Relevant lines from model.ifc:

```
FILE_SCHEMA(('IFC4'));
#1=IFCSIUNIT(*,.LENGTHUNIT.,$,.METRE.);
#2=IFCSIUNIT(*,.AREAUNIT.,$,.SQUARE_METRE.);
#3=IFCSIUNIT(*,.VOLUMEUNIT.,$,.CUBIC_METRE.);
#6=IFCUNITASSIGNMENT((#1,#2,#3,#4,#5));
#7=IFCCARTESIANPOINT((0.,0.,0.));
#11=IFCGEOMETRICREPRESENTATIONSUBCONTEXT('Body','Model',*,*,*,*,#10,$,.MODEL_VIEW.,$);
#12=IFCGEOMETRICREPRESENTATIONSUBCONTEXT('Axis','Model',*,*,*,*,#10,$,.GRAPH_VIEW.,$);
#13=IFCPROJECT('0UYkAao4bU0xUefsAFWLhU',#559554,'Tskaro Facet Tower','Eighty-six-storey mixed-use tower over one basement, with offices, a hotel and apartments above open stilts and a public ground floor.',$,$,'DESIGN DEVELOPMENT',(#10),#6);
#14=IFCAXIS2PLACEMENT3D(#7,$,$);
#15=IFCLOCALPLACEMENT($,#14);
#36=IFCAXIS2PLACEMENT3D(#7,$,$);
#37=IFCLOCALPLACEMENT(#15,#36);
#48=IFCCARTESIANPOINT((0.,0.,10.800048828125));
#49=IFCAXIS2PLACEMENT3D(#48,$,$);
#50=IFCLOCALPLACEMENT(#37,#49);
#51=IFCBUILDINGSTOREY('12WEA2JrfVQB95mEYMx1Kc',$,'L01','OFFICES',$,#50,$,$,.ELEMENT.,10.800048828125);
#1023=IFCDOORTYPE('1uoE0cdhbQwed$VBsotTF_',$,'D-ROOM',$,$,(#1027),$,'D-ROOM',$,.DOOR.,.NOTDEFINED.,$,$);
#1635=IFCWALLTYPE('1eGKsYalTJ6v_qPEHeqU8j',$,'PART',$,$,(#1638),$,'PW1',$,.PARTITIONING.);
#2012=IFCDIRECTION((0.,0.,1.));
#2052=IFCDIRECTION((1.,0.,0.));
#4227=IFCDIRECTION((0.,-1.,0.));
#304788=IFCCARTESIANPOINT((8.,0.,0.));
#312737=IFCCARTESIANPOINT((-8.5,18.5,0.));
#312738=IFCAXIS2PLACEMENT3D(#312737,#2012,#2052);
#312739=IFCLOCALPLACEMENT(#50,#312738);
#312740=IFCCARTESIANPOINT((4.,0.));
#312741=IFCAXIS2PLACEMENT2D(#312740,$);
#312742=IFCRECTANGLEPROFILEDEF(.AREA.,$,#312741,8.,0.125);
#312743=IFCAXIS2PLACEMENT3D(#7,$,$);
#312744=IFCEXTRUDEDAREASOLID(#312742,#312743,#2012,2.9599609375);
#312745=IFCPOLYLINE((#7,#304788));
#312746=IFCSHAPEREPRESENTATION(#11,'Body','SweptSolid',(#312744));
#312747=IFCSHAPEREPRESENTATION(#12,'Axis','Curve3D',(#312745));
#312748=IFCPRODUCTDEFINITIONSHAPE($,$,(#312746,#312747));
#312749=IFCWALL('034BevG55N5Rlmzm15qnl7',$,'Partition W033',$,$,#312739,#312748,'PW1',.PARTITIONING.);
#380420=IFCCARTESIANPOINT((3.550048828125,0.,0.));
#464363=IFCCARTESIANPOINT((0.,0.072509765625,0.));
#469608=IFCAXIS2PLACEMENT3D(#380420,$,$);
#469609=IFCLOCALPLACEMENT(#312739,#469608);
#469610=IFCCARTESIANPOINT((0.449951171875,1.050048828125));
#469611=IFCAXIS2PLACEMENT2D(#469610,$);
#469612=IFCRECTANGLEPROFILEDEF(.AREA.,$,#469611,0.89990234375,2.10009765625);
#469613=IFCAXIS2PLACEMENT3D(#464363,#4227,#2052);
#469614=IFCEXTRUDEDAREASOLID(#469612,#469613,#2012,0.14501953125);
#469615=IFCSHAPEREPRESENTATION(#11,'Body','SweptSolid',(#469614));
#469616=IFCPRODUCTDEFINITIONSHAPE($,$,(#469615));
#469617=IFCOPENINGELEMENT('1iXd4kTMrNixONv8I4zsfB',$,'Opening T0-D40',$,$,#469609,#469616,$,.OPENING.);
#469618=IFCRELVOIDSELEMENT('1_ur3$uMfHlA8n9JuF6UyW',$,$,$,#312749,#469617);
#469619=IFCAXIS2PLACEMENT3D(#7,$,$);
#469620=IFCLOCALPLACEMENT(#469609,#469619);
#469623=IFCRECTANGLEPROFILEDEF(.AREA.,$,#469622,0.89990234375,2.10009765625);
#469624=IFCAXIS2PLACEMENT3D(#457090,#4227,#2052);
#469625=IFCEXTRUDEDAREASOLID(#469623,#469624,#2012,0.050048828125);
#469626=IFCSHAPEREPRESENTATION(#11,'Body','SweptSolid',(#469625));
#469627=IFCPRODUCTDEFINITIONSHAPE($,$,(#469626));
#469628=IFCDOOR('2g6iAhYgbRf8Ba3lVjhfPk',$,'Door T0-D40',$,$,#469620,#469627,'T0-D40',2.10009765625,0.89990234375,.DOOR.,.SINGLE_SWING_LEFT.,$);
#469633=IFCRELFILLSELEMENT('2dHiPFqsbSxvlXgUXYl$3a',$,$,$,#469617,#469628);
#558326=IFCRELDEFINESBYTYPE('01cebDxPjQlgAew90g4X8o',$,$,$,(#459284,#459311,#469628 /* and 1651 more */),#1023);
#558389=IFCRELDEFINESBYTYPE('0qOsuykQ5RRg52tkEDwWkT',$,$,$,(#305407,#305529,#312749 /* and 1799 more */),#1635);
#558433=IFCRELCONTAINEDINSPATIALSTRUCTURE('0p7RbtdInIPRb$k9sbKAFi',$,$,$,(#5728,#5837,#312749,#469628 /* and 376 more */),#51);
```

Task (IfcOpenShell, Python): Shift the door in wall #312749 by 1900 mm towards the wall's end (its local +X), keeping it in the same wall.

```python
import ifcopenshell
import ifcopenshell.api.geometry
import ifcopenshell.util.placement
import ifcopenshell.util.unit

model = ifcopenshell.open("model.ifc")
unit_scale = ifcopenshell.util.unit.calculate_unit_scale(model)

door = model.by_guid("2g6iAhYgbRf8Ba3lVjhfPk")
opening = door.FillsVoids[0].RelatingOpeningElement
wall = opening.VoidsElements[0].RelatingBuildingElement

wall_matrix = ifcopenshell.util.placement.get_local_placement(wall.ObjectPlacement)
shift = wall_matrix[:3, 0] * 1.9 / unit_scale
before = ifcopenshell.util.placement.get_local_placement(door.ObjectPlacement)[:3, 3].copy()

# The door is placed relative to its opening, so it follows when the opening moves.
matrix = ifcopenshell.util.placement.get_local_placement(opening.ObjectPlacement)
matrix[:3, 3] += shift
ifcopenshell.api.geometry.edit_object_placement(
    model, product=opening, matrix=matrix, is_si=False, should_transform_children=True
)

after = ifcopenshell.util.placement.get_local_placement(door.ObjectPlacement)[:3, 3]
print("door moved by", (after - before).round(3) + 0.0)

model.write("model_updated.ifc")
```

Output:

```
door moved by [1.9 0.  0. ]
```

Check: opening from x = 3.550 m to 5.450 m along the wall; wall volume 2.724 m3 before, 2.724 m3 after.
